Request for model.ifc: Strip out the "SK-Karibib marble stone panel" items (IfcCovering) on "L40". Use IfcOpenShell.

First a look at what the model holds.

```python
import ifcopenshell
import ifcopenshell.util.element

model = ifcopenshell.open("model.ifc")
print(model.schema)
storey = next(s for s in model.by_type("IfcBuildingStorey") if s.Name == "L40")
coverings = [e for e in ifcopenshell.util.element.get_decomposition(storey) if e.is_a("IfcCovering")]
seen = {}
for e in coverings:
    element_type = ifcopenshell.util.element.get_type(e)
    name = element_type.Name if element_type not in (None, e) else None
    seen[name] = seen.get(name, 0) + 1
for name, count in sorted(seen.items(), key=str):
    print(count, "x", name)
```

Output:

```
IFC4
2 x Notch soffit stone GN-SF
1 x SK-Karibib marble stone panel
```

```python
import ifcopenshell
import ifcopenshell.api.root
import ifcopenshell.util.element

model = ifcopenshell.open("model.ifc")

storey = next(s for s in model.by_type("IfcBuildingStorey") if s.Name == "L40")
coverings = [e for e in ifcopenshell.util.element.get_decomposition(storey) if e.is_a("IfcCovering")]
targets = [e for e in coverings if (t := ifcopenshell.util.element.get_type(e)) not in (None, e) and t.Name == "SK-Karibib marble stone panel"]

for e in targets:
    ifcopenshell.api.root.remove_product(model, product=e)
print(len(targets), "removed")

model.write("model_updated.ifc")
```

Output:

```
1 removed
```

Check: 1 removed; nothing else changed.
